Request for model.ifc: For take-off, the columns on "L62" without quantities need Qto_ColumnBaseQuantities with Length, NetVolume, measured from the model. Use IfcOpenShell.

First a look at what the model holds.

```python
import ifcopenshell
import ifcopenshell.util.element
import ifcopenshell.util.unit

model = ifcopenshell.open("model.ifc")
print(model.schema)
for unit_type in ("LENGTHUNIT", "AREAUNIT", "VOLUMEUNIT"):
    print(unit_type, ifcopenshell.util.unit.calculate_unit_scale(model, unit_type))
storey = next(s for s in model.by_type("IfcBuildingStorey") if s.Name == "L62")
columns = [e for e in ifcopenshell.util.element.get_decomposition(storey) if e.is_a("IfcColumn")]
for e in sorted(columns, key=lambda e: e.id()):
    print(e.id(), e.is_a(), e.Name, list(ifcopenshell.util.element.get_psets(e, qtos_only=True)), sep=" | ")
```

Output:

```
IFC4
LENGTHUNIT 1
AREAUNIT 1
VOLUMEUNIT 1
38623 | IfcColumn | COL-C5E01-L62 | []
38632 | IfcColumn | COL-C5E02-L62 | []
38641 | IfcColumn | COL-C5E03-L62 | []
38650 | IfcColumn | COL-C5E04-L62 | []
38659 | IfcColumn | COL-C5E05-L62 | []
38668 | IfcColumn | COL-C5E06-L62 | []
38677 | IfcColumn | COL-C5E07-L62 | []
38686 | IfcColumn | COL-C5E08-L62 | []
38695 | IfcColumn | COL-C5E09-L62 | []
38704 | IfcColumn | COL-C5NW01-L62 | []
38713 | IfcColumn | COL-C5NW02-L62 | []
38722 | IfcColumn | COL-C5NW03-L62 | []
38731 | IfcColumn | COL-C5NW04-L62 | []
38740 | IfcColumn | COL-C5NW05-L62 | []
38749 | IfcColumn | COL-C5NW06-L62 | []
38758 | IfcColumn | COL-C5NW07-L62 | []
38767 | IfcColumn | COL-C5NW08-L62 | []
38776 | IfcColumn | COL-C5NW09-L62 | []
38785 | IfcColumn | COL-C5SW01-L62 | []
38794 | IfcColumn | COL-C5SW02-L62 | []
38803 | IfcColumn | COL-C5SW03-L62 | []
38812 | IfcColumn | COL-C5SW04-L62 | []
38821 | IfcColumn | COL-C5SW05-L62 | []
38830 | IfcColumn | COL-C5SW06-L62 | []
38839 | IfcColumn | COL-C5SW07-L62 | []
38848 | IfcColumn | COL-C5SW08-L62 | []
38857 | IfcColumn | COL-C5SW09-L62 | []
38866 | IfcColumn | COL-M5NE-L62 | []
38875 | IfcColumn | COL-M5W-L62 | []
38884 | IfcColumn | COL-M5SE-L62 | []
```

```python
import ifcopenshell
import ifcopenshell.api.pset
import ifcopenshell.geom
import ifcopenshell.util.element
import ifcopenshell.util.shape
import ifcopenshell.util.unit

model = ifcopenshell.open("model.ifc")
unit_scale = ifcopenshell.util.unit.calculate_unit_scale(model)
volume_scale = ifcopenshell.util.unit.calculate_unit_scale(model, "VOLUMEUNIT")
settings = ifcopenshell.geom.settings()

storey = next(s for s in model.by_type("IfcBuildingStorey") if s.Name == "L62")
columns = [e for e in ifcopenshell.util.element.get_decomposition(storey) if e.is_a("IfcColumn")]

for e in sorted(columns, key=lambda e: e.id()):
    if ifcopenshell.util.element.get_psets(e, qtos_only=True, should_inherit=False):
        continue
    # Geometry comes back in metres, in the element's own axes.
    shape = ifcopenshell.geom.create_shape(settings, e)
    values = {
        "Length": ifcopenshell.util.shape.get_z(shape.geometry) / unit_scale,
        "NetVolume": ifcopenshell.util.shape.get_volume(shape.geometry) / volume_scale,
    }
    qto = ifcopenshell.api.pset.add_qto(model, product=e, name="Qto_ColumnBaseQuantities")
    ifcopenshell.api.pset.edit_qto(model, qto=qto, properties=values)
    print(e.id(), {k: round(v, 3) for k, v in values.items()})

model.write("model_updated.ifc")
```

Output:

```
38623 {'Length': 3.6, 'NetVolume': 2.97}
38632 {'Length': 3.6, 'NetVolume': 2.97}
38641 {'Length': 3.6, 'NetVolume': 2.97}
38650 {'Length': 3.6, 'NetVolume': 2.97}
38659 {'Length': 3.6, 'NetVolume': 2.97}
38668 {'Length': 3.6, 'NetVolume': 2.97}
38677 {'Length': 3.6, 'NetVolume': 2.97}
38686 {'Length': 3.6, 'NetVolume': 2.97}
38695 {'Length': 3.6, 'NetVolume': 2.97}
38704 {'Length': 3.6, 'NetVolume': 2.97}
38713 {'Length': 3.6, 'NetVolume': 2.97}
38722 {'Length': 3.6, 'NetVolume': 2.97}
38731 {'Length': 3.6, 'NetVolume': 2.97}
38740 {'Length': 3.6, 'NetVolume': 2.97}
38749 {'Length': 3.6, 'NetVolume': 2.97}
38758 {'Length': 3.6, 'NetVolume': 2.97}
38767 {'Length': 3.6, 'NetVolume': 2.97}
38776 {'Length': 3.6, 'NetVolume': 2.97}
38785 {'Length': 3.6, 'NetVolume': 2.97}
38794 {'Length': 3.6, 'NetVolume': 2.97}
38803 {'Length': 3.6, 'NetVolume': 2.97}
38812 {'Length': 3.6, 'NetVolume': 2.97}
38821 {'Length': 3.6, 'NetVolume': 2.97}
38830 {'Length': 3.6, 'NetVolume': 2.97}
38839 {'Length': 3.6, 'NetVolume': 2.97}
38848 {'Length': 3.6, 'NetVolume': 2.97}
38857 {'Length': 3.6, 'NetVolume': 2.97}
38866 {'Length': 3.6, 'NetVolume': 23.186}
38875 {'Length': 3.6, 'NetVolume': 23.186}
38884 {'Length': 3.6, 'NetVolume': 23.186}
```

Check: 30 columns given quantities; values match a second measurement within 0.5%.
